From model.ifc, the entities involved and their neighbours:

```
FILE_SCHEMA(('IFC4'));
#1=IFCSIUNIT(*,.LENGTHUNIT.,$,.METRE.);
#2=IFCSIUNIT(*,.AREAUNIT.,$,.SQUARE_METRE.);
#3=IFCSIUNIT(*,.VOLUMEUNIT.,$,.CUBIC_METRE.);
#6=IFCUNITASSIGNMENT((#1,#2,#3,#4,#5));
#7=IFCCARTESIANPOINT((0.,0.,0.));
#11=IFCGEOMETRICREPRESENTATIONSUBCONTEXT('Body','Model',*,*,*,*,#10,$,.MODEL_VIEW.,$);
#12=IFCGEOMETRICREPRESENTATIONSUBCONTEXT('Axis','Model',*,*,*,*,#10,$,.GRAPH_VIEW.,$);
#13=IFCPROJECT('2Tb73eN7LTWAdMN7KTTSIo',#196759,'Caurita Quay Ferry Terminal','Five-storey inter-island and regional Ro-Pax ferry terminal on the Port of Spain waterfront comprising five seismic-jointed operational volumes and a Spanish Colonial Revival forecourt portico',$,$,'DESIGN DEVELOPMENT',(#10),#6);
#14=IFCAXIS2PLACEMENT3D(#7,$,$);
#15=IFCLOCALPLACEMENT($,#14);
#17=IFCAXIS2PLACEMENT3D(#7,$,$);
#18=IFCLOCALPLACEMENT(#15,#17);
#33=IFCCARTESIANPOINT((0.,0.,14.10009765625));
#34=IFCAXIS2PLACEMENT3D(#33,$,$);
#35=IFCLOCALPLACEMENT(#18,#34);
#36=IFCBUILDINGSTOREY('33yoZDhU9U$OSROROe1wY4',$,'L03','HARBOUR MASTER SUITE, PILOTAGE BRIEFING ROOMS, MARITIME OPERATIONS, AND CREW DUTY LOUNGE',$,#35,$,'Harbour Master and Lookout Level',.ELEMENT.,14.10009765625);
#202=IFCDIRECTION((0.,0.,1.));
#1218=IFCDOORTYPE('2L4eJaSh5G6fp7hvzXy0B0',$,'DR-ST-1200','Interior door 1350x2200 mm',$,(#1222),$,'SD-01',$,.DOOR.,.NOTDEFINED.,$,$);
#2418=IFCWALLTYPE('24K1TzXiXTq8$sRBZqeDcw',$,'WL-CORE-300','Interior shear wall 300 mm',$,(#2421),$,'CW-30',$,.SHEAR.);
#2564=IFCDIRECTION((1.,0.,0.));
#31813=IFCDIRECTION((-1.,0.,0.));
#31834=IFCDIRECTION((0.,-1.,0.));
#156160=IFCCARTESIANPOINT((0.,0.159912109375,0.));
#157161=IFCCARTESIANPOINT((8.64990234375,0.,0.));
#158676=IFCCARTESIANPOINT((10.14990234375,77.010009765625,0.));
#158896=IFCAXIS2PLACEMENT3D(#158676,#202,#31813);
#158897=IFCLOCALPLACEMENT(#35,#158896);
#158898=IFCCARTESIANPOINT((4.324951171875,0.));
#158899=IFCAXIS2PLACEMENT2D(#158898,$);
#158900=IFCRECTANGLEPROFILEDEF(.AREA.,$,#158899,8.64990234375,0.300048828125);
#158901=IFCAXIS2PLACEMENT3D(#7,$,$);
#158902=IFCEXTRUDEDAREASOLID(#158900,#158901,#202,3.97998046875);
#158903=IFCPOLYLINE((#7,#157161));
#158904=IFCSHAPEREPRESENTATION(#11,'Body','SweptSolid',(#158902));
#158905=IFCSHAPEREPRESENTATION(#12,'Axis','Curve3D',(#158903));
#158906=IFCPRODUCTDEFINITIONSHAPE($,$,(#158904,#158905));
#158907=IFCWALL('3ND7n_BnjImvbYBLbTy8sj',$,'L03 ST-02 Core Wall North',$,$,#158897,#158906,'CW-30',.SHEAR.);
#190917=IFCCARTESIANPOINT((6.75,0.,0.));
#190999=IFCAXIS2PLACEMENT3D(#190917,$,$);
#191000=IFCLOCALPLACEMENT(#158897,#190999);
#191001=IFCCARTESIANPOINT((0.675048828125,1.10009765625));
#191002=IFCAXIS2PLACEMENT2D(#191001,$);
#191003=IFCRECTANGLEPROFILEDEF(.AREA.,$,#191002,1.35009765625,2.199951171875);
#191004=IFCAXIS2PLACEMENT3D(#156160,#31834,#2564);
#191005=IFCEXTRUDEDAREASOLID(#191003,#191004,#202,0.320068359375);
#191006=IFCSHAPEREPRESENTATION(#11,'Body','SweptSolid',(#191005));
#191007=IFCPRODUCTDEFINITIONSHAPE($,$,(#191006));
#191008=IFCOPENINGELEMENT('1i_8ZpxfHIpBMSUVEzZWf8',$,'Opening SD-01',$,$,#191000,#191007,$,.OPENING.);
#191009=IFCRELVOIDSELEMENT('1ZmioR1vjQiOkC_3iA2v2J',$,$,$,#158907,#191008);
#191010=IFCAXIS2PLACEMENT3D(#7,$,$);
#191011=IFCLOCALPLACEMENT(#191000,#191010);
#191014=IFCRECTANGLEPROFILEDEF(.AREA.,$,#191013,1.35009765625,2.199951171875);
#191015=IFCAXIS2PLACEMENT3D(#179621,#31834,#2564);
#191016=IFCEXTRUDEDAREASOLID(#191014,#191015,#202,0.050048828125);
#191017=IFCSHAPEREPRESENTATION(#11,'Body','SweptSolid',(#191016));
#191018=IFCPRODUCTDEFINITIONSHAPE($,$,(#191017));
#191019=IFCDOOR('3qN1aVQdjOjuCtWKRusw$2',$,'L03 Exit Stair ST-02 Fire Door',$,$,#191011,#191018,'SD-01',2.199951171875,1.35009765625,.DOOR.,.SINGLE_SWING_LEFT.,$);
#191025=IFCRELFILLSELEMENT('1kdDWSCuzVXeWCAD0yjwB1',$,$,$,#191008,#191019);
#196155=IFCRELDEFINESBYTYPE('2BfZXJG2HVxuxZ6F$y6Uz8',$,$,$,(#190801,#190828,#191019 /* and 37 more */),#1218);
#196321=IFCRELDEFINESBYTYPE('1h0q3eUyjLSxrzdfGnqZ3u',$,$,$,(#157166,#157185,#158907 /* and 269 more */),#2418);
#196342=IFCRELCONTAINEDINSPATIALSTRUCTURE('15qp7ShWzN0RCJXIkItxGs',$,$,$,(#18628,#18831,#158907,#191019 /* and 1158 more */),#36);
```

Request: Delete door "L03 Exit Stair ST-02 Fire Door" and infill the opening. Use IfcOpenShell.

```python
import ifcopenshell
import ifcopenshell.api.feature
import ifcopenshell.api.root
import ifcopenshell.geom
import ifcopenshell.util.shape

model = ifcopenshell.open("model.ifc")
settings = ifcopenshell.geom.settings()


def volume(element):
    """Net volume in cubic metres, openings subtracted."""
    shape = ifcopenshell.geom.create_shape(settings, element)
    return ifcopenshell.util.shape.get_volume(shape.geometry)


door = model.by_id(191019)
opening = door.FillsVoids[0].RelatingOpeningElement
wall = opening.VoidsElements[0].RelatingBuildingElement
before = volume(wall)

ifcopenshell.api.root.remove_product(model, product=door)
ifcopenshell.api.feature.remove_feature(model, feature=opening)

after = volume(wall)

print(f"wall volume {before:.3f} -> {after:.3f} m3")

model.write("model_v2.ifc")
```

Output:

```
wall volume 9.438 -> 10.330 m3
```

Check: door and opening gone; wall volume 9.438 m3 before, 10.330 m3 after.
